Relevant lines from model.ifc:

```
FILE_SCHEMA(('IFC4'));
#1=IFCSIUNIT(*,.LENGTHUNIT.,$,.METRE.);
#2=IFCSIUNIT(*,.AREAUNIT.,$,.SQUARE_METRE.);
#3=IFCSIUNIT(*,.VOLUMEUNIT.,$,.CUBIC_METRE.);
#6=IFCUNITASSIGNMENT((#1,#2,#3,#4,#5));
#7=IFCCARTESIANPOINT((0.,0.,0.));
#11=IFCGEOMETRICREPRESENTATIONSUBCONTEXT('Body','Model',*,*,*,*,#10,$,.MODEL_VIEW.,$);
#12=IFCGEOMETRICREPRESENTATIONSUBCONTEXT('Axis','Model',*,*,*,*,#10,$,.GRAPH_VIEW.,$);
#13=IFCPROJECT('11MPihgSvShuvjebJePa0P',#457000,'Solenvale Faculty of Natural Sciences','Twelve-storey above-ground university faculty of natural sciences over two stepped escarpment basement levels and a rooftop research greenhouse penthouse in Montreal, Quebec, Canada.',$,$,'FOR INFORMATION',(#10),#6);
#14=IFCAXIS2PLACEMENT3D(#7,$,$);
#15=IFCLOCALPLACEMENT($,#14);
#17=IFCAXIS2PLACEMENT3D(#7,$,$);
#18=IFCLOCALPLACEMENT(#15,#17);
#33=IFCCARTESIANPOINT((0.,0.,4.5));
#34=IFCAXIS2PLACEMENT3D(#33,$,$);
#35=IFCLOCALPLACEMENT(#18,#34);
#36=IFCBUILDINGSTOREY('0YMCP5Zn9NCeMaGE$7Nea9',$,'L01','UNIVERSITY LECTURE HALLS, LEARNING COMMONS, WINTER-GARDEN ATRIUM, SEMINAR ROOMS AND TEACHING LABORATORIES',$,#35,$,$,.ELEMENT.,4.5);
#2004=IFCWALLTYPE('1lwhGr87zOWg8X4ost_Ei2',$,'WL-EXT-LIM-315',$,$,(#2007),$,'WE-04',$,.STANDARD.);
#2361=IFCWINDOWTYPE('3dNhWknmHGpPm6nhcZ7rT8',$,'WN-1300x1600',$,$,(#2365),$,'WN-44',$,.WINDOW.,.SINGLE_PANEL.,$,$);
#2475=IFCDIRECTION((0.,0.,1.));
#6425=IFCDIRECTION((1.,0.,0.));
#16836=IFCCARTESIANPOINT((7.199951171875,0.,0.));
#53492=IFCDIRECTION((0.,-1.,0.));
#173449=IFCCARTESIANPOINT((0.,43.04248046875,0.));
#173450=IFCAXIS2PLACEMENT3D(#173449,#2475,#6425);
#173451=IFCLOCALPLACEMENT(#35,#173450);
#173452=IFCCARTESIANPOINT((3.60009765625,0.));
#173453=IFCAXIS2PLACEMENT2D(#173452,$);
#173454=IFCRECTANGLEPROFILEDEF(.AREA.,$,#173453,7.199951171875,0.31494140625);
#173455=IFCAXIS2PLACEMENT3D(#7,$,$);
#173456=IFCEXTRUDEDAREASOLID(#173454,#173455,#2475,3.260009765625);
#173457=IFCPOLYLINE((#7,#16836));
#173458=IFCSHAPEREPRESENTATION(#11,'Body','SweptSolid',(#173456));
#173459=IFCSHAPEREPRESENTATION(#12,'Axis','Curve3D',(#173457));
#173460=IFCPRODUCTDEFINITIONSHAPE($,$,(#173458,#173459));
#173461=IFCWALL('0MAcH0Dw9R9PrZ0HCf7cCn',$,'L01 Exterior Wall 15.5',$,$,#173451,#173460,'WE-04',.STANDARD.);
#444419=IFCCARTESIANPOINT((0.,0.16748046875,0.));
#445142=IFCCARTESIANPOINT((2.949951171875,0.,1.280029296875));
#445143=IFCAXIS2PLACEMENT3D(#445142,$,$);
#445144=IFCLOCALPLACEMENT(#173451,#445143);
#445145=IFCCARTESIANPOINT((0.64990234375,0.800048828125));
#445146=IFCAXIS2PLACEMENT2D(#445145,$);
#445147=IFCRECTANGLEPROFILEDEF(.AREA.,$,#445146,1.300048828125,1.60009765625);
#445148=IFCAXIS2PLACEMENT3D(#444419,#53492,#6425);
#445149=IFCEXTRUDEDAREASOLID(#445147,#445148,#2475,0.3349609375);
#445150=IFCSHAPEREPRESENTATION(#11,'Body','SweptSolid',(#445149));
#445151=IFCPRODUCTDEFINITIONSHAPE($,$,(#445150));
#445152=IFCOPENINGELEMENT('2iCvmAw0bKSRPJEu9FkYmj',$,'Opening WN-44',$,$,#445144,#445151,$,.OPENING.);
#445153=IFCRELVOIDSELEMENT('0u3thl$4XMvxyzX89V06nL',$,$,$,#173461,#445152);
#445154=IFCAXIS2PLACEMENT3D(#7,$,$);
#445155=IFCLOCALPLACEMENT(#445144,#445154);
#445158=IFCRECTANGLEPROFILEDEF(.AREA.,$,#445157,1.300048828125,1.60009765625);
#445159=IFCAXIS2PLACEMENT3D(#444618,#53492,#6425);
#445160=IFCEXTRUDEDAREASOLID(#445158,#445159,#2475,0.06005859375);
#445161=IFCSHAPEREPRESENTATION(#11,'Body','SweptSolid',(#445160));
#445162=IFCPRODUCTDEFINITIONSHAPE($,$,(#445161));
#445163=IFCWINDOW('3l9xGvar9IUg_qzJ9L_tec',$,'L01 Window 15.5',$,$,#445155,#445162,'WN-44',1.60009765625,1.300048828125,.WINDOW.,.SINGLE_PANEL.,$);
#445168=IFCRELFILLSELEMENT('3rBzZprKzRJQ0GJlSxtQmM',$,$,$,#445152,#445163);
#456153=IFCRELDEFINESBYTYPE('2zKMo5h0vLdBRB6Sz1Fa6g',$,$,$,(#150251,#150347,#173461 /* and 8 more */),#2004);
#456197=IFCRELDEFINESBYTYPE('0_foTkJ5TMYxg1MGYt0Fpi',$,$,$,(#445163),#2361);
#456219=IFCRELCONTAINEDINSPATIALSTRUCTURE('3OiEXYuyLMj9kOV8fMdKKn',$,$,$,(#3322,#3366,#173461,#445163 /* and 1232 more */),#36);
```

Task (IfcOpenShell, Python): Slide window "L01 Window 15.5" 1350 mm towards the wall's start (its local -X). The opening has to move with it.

```python
import ifcopenshell
import ifcopenshell.api.geometry
import ifcopenshell.util.placement
import ifcopenshell.util.unit

model = ifcopenshell.open("model.ifc")
unit_scale = ifcopenshell.util.unit.calculate_unit_scale(model)

window = model.by_guid("3l9xGvar9IUg_qzJ9L_tec")
opening = window.FillsVoids[0].RelatingOpeningElement
wall = opening.VoidsElements[0].RelatingBuildingElement

wall_matrix = ifcopenshell.util.placement.get_local_placement(wall.ObjectPlacement)
shift = wall_matrix[:3, 0] * -1.35 / unit_scale
before = ifcopenshell.util.placement.get_local_placement(window.ObjectPlacement)[:3, 3].copy()

# The window is placed relative to its opening, so it follows when the opening moves.
matrix = ifcopenshell.util.placement.get_local_placement(opening.ObjectPlacement)
matrix[:3, 3] += shift
ifcopenshell.api.geometry.edit_object_placement(
    model, product=opening, matrix=matrix, is_si=False, should_transform_children=True
)

after = ifcopenshell.util.placement.get_local_placement(window.ObjectPlacement)[:3, 3]
print("window moved by", (after - before).round(3) + 0.0)

model.write("model_rev.ifc")
```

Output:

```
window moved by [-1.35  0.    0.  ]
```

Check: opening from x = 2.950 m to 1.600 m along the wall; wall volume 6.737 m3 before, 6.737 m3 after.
